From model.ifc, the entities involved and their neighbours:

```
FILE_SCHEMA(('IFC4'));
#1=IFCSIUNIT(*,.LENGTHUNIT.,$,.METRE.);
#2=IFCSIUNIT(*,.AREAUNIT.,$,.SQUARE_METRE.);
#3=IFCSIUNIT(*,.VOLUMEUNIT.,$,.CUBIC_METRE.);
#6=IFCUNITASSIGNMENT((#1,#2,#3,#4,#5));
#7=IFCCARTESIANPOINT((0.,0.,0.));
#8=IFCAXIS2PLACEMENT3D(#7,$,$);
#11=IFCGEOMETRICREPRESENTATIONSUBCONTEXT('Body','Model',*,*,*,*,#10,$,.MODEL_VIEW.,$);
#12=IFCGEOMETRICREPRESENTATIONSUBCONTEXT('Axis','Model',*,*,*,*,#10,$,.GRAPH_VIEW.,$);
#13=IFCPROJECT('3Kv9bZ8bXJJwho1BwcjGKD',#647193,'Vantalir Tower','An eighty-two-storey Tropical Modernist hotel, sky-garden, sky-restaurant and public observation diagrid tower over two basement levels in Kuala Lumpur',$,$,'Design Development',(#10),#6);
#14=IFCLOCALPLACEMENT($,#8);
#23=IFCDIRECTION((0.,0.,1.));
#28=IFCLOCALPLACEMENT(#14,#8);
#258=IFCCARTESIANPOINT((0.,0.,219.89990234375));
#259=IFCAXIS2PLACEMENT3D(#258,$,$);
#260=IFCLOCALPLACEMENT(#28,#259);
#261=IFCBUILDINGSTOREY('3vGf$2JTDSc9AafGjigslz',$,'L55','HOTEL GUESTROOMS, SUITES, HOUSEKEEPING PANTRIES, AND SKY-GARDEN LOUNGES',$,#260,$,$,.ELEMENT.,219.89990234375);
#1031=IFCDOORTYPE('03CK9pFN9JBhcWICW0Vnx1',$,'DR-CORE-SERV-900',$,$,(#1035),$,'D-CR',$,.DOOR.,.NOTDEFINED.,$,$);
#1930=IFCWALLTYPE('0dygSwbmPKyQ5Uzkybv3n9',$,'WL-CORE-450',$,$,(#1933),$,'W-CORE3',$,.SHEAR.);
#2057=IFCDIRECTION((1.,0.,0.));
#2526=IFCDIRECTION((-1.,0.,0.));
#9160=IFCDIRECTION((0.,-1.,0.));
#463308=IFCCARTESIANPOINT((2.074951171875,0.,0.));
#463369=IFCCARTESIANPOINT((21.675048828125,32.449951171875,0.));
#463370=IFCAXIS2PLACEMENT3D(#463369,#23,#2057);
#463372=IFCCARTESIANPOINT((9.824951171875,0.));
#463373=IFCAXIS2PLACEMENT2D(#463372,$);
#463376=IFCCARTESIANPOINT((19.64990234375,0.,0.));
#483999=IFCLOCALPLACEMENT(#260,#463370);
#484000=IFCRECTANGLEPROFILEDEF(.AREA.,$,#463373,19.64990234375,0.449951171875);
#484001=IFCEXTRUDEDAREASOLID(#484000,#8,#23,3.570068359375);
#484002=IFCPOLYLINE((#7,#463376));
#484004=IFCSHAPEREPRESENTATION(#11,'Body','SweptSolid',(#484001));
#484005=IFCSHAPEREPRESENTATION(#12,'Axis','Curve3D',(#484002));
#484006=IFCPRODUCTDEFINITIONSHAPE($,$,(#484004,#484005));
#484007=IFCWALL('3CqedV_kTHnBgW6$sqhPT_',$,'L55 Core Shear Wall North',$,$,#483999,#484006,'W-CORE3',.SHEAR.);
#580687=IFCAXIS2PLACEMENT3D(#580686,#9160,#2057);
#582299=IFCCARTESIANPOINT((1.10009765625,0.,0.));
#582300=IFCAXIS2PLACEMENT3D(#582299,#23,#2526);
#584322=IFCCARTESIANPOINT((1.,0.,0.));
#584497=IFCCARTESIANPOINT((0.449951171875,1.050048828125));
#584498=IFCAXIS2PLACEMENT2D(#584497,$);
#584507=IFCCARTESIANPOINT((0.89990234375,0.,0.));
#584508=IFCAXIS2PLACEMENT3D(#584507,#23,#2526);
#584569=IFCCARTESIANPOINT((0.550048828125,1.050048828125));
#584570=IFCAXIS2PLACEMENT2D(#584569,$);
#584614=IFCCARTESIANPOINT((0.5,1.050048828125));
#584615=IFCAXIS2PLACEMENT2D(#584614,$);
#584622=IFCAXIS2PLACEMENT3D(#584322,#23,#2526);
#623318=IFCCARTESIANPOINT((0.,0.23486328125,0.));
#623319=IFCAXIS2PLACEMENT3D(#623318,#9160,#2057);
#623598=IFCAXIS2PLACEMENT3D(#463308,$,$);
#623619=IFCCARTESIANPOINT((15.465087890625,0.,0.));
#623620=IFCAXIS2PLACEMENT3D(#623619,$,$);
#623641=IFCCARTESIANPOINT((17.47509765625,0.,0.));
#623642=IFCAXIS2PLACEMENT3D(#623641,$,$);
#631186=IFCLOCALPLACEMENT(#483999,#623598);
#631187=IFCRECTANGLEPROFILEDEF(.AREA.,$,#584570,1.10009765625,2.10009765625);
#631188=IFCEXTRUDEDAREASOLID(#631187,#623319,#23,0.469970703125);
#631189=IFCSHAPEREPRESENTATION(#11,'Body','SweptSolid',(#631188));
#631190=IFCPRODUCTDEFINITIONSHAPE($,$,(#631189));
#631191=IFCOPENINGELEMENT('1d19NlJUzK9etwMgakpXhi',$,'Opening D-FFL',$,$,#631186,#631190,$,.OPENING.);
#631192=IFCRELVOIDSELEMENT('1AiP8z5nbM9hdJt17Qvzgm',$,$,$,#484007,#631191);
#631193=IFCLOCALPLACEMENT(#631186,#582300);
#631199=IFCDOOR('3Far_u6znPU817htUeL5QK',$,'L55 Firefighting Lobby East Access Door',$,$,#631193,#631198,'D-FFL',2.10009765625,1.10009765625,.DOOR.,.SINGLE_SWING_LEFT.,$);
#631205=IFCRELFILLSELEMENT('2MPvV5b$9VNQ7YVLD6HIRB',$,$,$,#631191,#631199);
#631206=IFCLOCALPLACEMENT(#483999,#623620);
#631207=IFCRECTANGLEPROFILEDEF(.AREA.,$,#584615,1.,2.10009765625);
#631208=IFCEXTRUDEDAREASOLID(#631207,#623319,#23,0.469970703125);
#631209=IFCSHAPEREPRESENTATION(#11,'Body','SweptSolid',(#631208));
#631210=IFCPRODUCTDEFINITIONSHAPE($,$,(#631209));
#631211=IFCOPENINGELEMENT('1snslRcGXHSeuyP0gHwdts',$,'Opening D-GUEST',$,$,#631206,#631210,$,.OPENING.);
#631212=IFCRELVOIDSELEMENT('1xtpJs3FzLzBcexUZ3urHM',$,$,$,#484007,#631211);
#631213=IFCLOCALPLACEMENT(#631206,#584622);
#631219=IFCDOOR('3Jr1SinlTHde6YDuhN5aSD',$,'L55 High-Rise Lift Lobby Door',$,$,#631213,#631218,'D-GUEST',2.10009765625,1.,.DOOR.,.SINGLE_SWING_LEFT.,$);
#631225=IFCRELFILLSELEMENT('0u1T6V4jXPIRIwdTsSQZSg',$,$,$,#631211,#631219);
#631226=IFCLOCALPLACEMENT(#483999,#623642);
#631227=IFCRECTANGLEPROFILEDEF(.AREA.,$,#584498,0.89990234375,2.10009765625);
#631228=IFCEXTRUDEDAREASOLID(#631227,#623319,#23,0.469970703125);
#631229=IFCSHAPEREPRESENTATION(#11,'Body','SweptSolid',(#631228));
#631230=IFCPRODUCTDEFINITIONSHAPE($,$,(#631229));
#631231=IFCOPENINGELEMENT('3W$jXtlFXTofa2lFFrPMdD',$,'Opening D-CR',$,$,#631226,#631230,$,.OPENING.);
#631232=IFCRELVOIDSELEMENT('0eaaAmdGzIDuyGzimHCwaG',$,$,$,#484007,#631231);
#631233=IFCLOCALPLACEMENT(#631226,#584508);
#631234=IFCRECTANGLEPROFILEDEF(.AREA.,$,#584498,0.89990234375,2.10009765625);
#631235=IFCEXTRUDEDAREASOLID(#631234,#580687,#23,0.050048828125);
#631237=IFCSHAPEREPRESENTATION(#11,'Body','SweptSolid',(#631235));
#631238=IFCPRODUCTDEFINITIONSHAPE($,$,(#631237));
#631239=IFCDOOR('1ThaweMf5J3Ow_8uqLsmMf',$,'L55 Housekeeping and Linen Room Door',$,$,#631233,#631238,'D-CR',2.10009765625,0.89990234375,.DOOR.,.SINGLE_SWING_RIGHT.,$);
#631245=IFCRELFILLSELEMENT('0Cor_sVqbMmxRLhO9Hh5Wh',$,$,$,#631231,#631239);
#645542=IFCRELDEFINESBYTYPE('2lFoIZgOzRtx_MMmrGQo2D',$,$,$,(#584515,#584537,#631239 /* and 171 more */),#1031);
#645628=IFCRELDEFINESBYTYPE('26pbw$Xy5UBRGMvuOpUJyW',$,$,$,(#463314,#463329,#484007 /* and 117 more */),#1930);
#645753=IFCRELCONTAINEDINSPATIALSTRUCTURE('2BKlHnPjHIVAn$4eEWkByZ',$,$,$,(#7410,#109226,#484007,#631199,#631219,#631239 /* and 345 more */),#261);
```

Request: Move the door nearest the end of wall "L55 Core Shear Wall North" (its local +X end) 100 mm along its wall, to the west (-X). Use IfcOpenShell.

```python
import ifcopenshell
import ifcopenshell.api.geometry
import ifcopenshell.util.placement

model = ifcopenshell.open("model.ifc")

door = model.by_guid("1ThaweMf5J3Ow_8uqLsmMf")
opening = door.FillsVoids[0].RelatingOpeningElement
wall = opening.VoidsElements[0].RelatingBuildingElement

wall_matrix = ifcopenshell.util.placement.get_local_placement(wall.ObjectPlacement)
shift = wall_matrix[:3, 0] * -0.1
before = ifcopenshell.util.placement.get_local_placement(door.ObjectPlacement)[:3, 3].copy()

# The door is placed relative to its opening, so it follows when the opening moves.
matrix = ifcopenshell.util.placement.get_local_placement(opening.ObjectPlacement)
matrix[:3, 3] += shift
ifcopenshell.api.geometry.edit_object_placement(
    model, product=opening, matrix=matrix, is_si=False, should_transform_children=True
)

after = ifcopenshell.util.placement.get_local_placement(door.ObjectPlacement)[:3, 3]
print("door moved by", (after - before).round(3) + 0.0)

model.write("model_v2.ifc")
```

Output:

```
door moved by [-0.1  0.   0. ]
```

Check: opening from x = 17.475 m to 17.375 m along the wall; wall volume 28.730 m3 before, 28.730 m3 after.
